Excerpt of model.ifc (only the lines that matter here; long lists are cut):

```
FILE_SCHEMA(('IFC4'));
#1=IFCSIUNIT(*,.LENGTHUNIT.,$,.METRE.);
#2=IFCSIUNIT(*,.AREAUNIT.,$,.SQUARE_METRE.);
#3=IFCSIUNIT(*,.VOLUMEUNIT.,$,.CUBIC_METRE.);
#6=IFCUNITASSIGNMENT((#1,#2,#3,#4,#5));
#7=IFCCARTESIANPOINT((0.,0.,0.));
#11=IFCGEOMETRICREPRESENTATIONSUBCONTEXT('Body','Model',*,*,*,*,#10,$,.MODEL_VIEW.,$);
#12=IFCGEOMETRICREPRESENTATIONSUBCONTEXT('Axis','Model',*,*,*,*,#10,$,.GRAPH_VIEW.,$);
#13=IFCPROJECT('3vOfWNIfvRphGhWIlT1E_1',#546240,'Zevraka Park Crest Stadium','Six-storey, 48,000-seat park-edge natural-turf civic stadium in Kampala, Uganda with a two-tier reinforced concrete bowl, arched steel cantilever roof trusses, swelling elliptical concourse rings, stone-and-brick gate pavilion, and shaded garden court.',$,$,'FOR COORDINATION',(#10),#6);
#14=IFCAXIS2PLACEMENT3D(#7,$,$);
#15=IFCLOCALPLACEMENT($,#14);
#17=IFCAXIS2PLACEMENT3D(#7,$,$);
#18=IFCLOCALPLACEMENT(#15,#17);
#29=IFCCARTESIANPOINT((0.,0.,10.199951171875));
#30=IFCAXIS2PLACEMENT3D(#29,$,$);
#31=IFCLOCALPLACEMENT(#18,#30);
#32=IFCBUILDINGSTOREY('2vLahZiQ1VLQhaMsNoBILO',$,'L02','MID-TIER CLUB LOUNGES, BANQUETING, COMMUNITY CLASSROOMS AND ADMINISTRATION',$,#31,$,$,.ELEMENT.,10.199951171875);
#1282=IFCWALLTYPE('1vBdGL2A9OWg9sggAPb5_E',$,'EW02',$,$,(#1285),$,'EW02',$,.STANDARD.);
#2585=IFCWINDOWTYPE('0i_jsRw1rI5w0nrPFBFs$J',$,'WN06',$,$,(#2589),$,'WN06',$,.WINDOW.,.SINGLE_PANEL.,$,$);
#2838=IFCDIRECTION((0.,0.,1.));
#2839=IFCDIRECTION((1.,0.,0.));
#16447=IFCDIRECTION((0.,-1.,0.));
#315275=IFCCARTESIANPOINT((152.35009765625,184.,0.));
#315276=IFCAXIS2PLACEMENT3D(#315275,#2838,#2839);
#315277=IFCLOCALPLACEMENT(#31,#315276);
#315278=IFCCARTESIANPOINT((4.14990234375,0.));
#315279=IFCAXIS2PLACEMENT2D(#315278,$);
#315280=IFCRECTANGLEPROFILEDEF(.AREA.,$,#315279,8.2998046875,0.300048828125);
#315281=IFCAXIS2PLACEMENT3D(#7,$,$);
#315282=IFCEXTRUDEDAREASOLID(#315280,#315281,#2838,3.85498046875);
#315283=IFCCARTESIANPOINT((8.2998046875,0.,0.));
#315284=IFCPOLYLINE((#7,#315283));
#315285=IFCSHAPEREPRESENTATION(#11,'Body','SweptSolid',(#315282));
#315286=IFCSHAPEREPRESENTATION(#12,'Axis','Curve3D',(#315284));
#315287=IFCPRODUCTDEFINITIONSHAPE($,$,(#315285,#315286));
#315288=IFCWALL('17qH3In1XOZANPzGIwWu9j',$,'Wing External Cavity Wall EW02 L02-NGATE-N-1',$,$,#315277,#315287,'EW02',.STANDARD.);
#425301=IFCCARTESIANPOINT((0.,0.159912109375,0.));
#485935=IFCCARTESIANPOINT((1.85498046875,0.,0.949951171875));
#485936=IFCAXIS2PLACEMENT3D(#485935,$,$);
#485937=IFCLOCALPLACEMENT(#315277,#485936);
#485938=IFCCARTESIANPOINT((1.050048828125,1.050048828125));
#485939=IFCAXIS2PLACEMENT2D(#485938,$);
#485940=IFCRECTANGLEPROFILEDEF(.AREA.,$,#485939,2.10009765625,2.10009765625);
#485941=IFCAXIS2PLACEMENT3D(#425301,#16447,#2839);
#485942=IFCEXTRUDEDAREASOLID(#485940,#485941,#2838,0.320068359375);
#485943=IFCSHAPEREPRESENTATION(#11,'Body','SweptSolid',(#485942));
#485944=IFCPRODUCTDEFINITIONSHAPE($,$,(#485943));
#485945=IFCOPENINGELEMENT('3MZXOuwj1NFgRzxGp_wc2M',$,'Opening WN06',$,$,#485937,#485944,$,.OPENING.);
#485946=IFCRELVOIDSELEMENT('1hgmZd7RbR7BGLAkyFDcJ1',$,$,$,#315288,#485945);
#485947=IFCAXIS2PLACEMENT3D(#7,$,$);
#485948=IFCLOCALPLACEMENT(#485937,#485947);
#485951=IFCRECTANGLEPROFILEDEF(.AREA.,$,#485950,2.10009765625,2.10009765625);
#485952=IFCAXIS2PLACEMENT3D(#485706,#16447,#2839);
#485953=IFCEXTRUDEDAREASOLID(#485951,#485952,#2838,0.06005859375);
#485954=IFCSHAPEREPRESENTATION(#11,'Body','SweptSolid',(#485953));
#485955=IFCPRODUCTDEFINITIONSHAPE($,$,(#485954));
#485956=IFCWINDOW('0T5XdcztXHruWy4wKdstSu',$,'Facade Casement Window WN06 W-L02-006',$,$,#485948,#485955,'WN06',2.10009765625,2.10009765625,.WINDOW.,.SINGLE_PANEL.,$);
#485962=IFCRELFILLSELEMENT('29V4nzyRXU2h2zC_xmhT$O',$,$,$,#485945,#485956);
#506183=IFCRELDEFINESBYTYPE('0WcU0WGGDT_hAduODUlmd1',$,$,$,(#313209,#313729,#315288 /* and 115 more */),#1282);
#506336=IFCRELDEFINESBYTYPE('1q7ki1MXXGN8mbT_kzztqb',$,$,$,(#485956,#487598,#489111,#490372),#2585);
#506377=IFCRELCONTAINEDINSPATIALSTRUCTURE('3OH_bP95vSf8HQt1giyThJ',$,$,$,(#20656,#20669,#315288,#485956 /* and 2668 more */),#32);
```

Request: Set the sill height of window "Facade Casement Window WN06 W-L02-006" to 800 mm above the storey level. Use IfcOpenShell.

```python
import numpy as np
import ifcopenshell
import ifcopenshell.api.geometry
import ifcopenshell.geom
import ifcopenshell.util.element
import ifcopenshell.util.placement
import ifcopenshell.util.shape
import ifcopenshell.util.unit

model = ifcopenshell.open("model.ifc")
unit_scale = ifcopenshell.util.unit.calculate_unit_scale(model)

window = model.by_guid("0T5XdcztXHruWy4wKdstSu")
opening = window.FillsVoids[0].RelatingOpeningElement
storey = ifcopenshell.util.element.get_container(window, ifc_class="IfcBuildingStorey")
level = ifcopenshell.util.placement.get_local_placement(storey.ObjectPlacement)[2, 3]

# The opening's origin need not be at the sill, so measure its lowest point.
shape = ifcopenshell.geom.create_shape(ifcopenshell.geom.settings(), opening)
bottom = ifcopenshell.util.shape.get_shape_bottom_elevation(shape, shape.geometry) / unit_scale
dz = level + 0.8 / unit_scale - bottom

shift = np.array([0.0, 0.0, dz])
# The window is placed relative to its opening, so it follows when the opening moves.
matrix = ifcopenshell.util.placement.get_local_placement(opening.ObjectPlacement)
matrix[:3, 3] += shift
ifcopenshell.api.geometry.edit_object_placement(
    model, product=opening, matrix=matrix, is_si=False, should_transform_children=True
)

print(f"moved by {dz * unit_scale:+.3f} m")

model.write("model_edited.ifc")
```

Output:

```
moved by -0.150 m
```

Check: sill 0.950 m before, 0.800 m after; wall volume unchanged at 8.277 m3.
